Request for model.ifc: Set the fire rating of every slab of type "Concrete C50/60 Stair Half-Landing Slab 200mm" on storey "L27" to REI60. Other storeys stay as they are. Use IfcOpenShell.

First a look at what the model holds.

```python
import ifcopenshell
import ifcopenshell.util.element

model = ifcopenshell.open("model.ifc")
print(model.schema)
storey = next(s for s in model.by_type("IfcBuildingStorey") if s.Name == "L27")
slabs = [e for e in ifcopenshell.util.element.get_decomposition(storey) if e.is_a("IfcSlab")]
seen = {}
for e in slabs:
    element_type = ifcopenshell.util.element.get_type(e)
    key = (element_type.Name if element_type != e and element_type else None, ifcopenshell.util.element.get_pset(e, "Pset_SlabCommon", "FireRating"))
    seen[key] = seen.get(key, 0) + 1
for (name, value), count in sorted(seen.items(), key=str):
    print(count, "x", name, "|", value)
```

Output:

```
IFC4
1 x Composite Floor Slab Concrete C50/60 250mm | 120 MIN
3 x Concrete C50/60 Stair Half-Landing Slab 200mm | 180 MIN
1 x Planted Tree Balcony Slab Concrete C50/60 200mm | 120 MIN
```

```python
import ifcopenshell
import ifcopenshell.api.pset
import ifcopenshell.util.element

model = ifcopenshell.open("model.ifc")

storey = next(s for s in model.by_type("IfcBuildingStorey") if s.Name == "L27")
slabs = [e for e in ifcopenshell.util.element.get_decomposition(storey) if e.is_a("IfcSlab")]

count = 0
for e in slabs:
    element_type = ifcopenshell.util.element.get_type(e)
    if element_type in (None, e) or element_type.Name != "Concrete C50/60 Stair Half-Landing Slab 200mm":
        continue
    # add_pset returns the element's existing set when there is one.
    pset = ifcopenshell.api.pset.add_pset(model, product=e, name="Pset_SlabCommon")
    ifcopenshell.api.pset.edit_pset(model, pset=pset, properties={"FireRating": "REI60"})
    count += 1

print(count, "slabs updated")

model.write("model-out.ifc")
```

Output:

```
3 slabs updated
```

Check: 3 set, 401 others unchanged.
